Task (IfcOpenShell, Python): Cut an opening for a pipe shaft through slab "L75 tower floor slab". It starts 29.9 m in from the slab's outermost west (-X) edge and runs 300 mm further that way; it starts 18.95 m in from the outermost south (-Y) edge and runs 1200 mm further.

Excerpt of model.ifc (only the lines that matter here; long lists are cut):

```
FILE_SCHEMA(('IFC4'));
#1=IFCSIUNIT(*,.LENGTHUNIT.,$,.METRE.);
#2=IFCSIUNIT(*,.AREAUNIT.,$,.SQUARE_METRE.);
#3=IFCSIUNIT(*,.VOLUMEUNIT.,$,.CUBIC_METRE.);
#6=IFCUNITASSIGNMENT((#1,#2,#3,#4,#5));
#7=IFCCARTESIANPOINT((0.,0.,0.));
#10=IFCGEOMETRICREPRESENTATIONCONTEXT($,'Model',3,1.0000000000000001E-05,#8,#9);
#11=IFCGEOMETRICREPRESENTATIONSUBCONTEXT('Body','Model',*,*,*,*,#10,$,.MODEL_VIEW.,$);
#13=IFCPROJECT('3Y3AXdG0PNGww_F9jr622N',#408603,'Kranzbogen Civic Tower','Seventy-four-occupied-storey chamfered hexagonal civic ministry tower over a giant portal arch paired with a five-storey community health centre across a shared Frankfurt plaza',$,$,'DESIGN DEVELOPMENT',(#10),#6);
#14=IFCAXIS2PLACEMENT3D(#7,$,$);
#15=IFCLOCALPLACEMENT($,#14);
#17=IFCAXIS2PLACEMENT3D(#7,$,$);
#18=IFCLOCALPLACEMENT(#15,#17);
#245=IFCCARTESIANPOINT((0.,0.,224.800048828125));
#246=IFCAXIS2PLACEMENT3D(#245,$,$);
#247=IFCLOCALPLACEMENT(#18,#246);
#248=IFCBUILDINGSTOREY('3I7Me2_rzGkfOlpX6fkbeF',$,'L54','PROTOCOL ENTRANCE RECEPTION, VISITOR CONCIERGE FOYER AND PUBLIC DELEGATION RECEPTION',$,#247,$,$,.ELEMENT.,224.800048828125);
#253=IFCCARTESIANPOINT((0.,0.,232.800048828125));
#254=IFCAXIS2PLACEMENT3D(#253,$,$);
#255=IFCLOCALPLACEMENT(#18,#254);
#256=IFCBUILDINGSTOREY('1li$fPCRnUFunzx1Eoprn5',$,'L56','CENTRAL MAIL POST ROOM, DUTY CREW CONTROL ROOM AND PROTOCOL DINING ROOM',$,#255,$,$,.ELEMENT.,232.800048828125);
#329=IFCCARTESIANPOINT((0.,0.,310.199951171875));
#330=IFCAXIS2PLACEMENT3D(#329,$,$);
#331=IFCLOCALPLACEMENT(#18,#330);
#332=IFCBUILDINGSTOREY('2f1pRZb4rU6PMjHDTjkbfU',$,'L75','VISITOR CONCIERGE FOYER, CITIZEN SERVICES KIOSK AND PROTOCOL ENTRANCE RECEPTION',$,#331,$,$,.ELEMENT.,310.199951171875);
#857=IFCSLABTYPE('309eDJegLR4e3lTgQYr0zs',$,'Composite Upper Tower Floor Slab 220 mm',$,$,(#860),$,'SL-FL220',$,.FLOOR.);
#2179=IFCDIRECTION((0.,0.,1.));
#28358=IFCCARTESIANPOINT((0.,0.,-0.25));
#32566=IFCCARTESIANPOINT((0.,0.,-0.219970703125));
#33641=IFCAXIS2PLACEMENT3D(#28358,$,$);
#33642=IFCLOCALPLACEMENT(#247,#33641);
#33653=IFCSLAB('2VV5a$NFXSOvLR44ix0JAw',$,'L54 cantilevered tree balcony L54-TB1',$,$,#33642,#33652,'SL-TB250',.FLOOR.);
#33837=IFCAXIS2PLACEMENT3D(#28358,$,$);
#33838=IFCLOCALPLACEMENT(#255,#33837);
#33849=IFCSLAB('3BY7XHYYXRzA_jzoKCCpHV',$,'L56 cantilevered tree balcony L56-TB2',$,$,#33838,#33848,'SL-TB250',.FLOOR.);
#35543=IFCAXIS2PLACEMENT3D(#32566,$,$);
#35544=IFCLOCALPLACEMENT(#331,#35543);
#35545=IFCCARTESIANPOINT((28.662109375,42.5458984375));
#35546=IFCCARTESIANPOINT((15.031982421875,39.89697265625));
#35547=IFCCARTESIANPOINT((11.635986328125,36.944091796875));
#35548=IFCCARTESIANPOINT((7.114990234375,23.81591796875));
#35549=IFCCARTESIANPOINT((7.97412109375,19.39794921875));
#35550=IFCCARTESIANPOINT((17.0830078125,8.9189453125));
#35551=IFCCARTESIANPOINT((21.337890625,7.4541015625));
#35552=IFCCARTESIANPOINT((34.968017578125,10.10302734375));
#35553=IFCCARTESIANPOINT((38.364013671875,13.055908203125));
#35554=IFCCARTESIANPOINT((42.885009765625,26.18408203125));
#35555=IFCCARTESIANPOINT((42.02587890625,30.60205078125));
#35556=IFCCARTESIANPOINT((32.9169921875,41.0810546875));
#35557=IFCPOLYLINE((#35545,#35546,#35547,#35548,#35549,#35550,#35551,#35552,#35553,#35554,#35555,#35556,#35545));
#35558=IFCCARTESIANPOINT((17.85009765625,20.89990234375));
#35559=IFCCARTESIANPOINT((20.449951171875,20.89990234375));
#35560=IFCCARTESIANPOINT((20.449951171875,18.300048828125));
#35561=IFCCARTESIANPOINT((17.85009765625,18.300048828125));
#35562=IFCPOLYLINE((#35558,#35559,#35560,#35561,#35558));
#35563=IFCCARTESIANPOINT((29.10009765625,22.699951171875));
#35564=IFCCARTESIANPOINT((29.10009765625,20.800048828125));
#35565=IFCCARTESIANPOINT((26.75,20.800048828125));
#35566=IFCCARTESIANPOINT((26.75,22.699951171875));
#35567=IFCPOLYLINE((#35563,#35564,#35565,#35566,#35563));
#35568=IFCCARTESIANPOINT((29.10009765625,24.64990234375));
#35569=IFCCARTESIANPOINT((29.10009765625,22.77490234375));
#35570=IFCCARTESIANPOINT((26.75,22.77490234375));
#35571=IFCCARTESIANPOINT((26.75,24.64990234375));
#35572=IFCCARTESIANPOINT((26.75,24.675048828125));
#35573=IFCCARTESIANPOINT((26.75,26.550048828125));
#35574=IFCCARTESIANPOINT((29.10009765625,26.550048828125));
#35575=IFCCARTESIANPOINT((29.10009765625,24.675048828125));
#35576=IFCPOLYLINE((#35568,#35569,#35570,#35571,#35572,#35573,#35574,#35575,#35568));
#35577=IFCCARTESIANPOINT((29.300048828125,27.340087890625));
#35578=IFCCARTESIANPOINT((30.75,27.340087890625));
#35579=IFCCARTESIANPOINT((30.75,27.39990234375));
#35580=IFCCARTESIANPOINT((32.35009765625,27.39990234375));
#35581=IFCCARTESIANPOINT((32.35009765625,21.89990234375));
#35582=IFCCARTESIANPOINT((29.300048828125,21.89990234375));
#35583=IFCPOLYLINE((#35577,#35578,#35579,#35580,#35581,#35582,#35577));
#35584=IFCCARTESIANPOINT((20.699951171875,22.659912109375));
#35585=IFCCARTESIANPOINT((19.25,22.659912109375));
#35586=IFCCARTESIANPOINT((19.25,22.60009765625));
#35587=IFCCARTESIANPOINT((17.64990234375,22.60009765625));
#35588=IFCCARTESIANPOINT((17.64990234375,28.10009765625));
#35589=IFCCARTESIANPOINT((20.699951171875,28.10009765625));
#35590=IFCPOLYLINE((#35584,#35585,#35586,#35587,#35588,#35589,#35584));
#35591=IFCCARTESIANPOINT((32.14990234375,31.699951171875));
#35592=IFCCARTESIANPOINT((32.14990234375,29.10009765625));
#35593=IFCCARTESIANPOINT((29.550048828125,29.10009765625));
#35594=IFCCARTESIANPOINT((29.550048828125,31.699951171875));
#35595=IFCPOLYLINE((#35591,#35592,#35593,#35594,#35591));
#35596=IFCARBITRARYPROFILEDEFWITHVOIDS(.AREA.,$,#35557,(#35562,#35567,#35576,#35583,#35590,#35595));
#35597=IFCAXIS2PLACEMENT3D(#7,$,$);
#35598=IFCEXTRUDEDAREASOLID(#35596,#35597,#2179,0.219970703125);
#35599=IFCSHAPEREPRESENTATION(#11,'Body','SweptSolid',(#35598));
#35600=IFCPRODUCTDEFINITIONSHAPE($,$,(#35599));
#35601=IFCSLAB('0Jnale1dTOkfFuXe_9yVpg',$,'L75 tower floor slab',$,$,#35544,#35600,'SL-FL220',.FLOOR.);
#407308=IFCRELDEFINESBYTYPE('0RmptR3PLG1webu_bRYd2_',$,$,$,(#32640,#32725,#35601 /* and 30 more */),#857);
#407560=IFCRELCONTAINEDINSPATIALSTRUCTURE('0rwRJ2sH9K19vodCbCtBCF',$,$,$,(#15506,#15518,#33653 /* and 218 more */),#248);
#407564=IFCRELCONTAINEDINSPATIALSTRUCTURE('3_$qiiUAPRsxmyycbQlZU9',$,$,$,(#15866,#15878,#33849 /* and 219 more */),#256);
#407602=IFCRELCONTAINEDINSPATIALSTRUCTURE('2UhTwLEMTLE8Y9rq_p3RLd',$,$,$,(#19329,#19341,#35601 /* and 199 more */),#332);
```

```python
import numpy as np
import ifcopenshell
import ifcopenshell.api.feature
import ifcopenshell.api.geometry
import ifcopenshell.api.root
import ifcopenshell.geom
import ifcopenshell.util.placement
import ifcopenshell.util.representation
import ifcopenshell.util.shape
import ifcopenshell.util.unit

model = ifcopenshell.open("model.ifc")
unit_scale = ifcopenshell.util.unit.calculate_unit_scale(model)
settings = ifcopenshell.geom.settings()


def volume(element):
    """Net volume in cubic metres, openings subtracted."""
    shape = ifcopenshell.geom.create_shape(settings, element)
    return ifcopenshell.util.shape.get_volume(shape.geometry)


slab = model.by_guid("0Jnale1dTOkfFuXe_9yVpg")
before = volume(slab)

# Extent in the slab's own axes, in metres. The edges named are its -X and -Y sides.
slab_shape = ifcopenshell.geom.create_shape(settings, slab)
vertices = ifcopenshell.util.shape.get_vertices(slab_shape.geometry)
x_min, y_min, bottom = vertices.min(axis=0)
top = vertices[:, 2].max()

opening = ifcopenshell.api.root.create_entity(model, ifc_class="IfcOpeningElement", name="Pipe shaft opening", predefined_type="OPENING")
context = ifcopenshell.util.representation.get_context(model, "Model", "Body", "MODEL_VIEW")
width, depth = 0.3, 1.2
outline = [(0.0, 0.0), (width, 0.0), (width, depth), (0.0, depth), (0.0, 0.0)]
# Overshoot both faces by 50 mm so the cut is clean.
shape = ifcopenshell.api.geometry.add_slab_representation(
    model, context=context, depth=top - bottom + 0.1, polyline=outline
)
ifcopenshell.api.geometry.assign_representation(model, product=opening, representation=shape)

matrix = ifcopenshell.util.placement.get_local_placement(slab.ObjectPlacement)
matrix[:, 3] = matrix @ np.append(np.array([x_min + 29.9, y_min + 18.95, bottom - 0.05]) / unit_scale, 1.0)
ifcopenshell.api.geometry.edit_object_placement(model, product=opening, matrix=matrix, is_si=False)
ifcopenshell.api.feature.add_feature(model, feature=opening, element=slab)

after = volume(slab)

print(f"slab volume {before:.3f} -> {after:.3f} m3")

model.write("model_updated.ifc")
```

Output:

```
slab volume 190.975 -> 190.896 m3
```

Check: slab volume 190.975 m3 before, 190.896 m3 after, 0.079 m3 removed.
